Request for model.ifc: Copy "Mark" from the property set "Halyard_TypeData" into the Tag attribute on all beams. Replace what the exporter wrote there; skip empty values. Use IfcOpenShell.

First a look at what the model holds.

```python
import ifcopenshell
import ifcopenshell.util.element

model = ifcopenshell.open("model.ifc")
print(model.schema)
beams = model.by_type("IfcBeam")
print(len(beams), "beams")
for e in beams[:8]:
    source = ifcopenshell.util.element.get_pset(e, "Halyard_TypeData", "Mark")
    target = e.Tag
    print(e.id(), repr(source), repr(target), sep=" | ")
```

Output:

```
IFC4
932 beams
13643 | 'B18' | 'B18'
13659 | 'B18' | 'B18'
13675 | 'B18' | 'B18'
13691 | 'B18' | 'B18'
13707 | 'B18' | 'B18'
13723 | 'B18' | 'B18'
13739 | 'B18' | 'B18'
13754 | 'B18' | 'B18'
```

```python
import ifcopenshell
import ifcopenshell.util.element

model = ifcopenshell.open("model.ifc")

count = 0
for e in model.by_type("IfcBeam"):
    value = ifcopenshell.util.element.get_pset(e, "Halyard_TypeData", "Mark")
    current = e.Tag
    if not value or not value.strip() or current == value:
        continue
    e.Tag = value
    count += 1

print(count, "beams updated")

model.write("model_v2.ifc")
```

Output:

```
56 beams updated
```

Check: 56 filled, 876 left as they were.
